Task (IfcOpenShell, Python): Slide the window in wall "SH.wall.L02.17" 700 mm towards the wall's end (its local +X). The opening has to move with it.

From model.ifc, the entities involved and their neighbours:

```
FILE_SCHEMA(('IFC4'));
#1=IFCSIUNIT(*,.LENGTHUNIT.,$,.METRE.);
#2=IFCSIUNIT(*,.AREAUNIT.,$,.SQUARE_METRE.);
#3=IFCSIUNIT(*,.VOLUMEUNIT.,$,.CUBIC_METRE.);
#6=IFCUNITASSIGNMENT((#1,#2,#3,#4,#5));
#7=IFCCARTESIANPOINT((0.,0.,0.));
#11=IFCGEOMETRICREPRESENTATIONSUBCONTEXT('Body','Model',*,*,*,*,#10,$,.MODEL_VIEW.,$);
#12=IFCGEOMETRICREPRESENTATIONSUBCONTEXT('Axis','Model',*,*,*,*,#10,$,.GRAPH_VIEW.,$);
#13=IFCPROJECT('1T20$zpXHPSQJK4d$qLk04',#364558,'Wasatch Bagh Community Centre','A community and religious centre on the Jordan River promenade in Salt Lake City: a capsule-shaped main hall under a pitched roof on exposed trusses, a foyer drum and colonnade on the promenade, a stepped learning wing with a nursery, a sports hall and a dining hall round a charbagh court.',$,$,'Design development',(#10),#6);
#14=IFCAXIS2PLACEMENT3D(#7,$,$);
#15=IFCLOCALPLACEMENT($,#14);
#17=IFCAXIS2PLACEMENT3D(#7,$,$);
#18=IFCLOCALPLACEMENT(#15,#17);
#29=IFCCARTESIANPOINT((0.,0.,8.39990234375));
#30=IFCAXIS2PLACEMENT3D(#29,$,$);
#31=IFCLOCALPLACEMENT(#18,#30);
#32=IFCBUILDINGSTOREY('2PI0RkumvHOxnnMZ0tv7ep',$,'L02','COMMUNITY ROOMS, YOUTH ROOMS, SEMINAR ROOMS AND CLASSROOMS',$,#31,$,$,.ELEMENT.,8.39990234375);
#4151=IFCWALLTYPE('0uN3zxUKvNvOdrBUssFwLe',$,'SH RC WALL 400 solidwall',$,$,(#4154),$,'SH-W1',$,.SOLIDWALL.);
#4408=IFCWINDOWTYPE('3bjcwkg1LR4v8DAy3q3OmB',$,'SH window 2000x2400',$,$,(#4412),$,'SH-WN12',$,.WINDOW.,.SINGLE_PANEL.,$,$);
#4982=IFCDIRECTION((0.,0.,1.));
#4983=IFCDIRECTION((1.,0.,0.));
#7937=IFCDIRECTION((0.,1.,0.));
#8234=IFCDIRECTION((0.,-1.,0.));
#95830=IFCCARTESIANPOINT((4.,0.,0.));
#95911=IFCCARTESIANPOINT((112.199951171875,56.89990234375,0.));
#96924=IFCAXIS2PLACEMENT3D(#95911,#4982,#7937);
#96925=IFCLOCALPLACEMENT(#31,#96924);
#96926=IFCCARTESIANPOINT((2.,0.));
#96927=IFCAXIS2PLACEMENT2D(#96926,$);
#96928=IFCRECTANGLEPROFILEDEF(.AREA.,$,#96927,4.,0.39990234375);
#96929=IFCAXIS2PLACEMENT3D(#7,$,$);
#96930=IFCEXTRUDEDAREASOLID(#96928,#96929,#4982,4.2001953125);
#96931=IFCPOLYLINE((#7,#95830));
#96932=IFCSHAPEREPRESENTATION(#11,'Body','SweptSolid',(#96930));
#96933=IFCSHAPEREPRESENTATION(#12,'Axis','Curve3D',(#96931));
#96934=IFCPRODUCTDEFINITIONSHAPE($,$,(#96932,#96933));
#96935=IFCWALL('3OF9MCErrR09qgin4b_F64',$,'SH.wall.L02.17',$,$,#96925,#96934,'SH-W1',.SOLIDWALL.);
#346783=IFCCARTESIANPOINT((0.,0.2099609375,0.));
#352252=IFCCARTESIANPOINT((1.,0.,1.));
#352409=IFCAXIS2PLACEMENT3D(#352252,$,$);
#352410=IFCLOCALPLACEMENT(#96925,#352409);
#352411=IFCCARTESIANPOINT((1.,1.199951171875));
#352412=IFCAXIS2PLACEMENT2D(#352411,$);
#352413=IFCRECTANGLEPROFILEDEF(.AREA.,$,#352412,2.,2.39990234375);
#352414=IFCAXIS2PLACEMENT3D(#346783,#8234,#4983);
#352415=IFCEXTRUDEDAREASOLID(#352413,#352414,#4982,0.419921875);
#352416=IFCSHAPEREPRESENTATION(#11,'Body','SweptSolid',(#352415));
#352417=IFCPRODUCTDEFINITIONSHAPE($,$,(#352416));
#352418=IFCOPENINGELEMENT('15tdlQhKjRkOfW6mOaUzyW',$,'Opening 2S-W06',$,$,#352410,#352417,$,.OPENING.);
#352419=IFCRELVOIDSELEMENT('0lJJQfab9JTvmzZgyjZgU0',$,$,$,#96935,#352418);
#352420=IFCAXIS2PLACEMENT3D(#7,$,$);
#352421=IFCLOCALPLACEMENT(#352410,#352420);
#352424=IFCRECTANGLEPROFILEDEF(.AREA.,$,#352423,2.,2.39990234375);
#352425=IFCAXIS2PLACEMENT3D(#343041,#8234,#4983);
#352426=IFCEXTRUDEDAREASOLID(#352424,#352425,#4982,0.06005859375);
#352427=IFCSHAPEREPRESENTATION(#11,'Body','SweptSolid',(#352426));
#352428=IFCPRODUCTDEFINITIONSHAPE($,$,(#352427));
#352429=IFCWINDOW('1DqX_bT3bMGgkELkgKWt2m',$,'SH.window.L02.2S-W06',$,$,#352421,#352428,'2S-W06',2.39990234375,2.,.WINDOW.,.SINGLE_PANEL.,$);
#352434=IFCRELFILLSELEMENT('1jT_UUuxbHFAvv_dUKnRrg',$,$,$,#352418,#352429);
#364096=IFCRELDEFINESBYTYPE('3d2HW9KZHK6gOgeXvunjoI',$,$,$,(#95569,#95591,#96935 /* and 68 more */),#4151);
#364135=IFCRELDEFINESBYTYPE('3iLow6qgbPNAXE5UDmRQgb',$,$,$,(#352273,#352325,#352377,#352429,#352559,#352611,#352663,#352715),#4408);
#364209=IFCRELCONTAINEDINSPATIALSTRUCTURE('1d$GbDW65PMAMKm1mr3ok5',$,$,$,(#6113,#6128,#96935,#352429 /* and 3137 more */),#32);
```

```python
import ifcopenshell
import ifcopenshell.api.geometry
import ifcopenshell.util.placement
import ifcopenshell.util.unit

model = ifcopenshell.open("model.ifc")
unit_scale = ifcopenshell.util.unit.calculate_unit_scale(model)

window = model.by_guid("1DqX_bT3bMGgkELkgKWt2m")
opening = window.FillsVoids[0].RelatingOpeningElement
wall = opening.VoidsElements[0].RelatingBuildingElement

wall_matrix = ifcopenshell.util.placement.get_local_placement(wall.ObjectPlacement)
shift = wall_matrix[:3, 0] * 0.7 / unit_scale
before = ifcopenshell.util.placement.get_local_placement(window.ObjectPlacement)[:3, 3].copy()

# The window is placed relative to its opening, so it follows when the opening moves.
matrix = ifcopenshell.util.placement.get_local_placement(opening.ObjectPlacement)
matrix[:3, 3] += shift
ifcopenshell.api.geometry.edit_object_placement(
    model, product=opening, matrix=matrix, is_si=False, should_transform_children=True
)

after = ifcopenshell.util.placement.get_local_placement(window.ObjectPlacement)[:3, 3]
print("window moved by", (after - before).round(3) + 0.0)

model.write("model_edited.ifc")
```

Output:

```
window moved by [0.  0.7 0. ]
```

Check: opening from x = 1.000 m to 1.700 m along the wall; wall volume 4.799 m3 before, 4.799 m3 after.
